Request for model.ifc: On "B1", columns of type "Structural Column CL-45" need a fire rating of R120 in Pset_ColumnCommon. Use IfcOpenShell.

First a look at what the model holds.

```python
import ifcopenshell
import ifcopenshell.util.element

model = ifcopenshell.open("model.ifc")
print(model.schema)
storey = next(s for s in model.by_type("IfcBuildingStorey") if s.Name == "B1")
columns = [e for e in ifcopenshell.util.element.get_decomposition(storey) if e.is_a("IfcColumn")]
seen = {}
for e in columns:
    element_type = ifcopenshell.util.element.get_type(e)
    key = (element_type.Name if element_type != e and element_type else None, ifcopenshell.util.element.get_pset(e, "Pset_ColumnCommon", "FireRating"))
    seen[key] = seen.get(key, 0) + 1
for (name, value), count in sorted(seen.items(), key=str):
    print(count, "x", name, "|", value)
```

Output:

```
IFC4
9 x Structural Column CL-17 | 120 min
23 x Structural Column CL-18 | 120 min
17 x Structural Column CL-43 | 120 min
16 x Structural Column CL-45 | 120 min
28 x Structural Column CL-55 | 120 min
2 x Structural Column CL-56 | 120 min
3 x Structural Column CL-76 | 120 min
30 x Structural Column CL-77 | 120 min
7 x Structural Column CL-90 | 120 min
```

```python
import ifcopenshell
import ifcopenshell.api.pset
import ifcopenshell.util.element

model = ifcopenshell.open("model.ifc")

storey = next(s for s in model.by_type("IfcBuildingStorey") if s.Name == "B1")
columns = [e for e in ifcopenshell.util.element.get_decomposition(storey) if e.is_a("IfcColumn")]

count = 0
for e in columns:
    element_type = ifcopenshell.util.element.get_type(e)
    if element_type in (None, e) or element_type.Name != "Structural Column CL-45":
        continue
    # add_pset returns the element's existing set when there is one.
    pset = ifcopenshell.api.pset.add_pset(model, product=e, name="Pset_ColumnCommon")
    ifcopenshell.api.pset.edit_pset(model, pset=pset, properties={"FireRating": "R120"})
    count += 1

print(count, "columns updated")

model.write("model_edited.ifc")
```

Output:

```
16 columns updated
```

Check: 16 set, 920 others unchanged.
